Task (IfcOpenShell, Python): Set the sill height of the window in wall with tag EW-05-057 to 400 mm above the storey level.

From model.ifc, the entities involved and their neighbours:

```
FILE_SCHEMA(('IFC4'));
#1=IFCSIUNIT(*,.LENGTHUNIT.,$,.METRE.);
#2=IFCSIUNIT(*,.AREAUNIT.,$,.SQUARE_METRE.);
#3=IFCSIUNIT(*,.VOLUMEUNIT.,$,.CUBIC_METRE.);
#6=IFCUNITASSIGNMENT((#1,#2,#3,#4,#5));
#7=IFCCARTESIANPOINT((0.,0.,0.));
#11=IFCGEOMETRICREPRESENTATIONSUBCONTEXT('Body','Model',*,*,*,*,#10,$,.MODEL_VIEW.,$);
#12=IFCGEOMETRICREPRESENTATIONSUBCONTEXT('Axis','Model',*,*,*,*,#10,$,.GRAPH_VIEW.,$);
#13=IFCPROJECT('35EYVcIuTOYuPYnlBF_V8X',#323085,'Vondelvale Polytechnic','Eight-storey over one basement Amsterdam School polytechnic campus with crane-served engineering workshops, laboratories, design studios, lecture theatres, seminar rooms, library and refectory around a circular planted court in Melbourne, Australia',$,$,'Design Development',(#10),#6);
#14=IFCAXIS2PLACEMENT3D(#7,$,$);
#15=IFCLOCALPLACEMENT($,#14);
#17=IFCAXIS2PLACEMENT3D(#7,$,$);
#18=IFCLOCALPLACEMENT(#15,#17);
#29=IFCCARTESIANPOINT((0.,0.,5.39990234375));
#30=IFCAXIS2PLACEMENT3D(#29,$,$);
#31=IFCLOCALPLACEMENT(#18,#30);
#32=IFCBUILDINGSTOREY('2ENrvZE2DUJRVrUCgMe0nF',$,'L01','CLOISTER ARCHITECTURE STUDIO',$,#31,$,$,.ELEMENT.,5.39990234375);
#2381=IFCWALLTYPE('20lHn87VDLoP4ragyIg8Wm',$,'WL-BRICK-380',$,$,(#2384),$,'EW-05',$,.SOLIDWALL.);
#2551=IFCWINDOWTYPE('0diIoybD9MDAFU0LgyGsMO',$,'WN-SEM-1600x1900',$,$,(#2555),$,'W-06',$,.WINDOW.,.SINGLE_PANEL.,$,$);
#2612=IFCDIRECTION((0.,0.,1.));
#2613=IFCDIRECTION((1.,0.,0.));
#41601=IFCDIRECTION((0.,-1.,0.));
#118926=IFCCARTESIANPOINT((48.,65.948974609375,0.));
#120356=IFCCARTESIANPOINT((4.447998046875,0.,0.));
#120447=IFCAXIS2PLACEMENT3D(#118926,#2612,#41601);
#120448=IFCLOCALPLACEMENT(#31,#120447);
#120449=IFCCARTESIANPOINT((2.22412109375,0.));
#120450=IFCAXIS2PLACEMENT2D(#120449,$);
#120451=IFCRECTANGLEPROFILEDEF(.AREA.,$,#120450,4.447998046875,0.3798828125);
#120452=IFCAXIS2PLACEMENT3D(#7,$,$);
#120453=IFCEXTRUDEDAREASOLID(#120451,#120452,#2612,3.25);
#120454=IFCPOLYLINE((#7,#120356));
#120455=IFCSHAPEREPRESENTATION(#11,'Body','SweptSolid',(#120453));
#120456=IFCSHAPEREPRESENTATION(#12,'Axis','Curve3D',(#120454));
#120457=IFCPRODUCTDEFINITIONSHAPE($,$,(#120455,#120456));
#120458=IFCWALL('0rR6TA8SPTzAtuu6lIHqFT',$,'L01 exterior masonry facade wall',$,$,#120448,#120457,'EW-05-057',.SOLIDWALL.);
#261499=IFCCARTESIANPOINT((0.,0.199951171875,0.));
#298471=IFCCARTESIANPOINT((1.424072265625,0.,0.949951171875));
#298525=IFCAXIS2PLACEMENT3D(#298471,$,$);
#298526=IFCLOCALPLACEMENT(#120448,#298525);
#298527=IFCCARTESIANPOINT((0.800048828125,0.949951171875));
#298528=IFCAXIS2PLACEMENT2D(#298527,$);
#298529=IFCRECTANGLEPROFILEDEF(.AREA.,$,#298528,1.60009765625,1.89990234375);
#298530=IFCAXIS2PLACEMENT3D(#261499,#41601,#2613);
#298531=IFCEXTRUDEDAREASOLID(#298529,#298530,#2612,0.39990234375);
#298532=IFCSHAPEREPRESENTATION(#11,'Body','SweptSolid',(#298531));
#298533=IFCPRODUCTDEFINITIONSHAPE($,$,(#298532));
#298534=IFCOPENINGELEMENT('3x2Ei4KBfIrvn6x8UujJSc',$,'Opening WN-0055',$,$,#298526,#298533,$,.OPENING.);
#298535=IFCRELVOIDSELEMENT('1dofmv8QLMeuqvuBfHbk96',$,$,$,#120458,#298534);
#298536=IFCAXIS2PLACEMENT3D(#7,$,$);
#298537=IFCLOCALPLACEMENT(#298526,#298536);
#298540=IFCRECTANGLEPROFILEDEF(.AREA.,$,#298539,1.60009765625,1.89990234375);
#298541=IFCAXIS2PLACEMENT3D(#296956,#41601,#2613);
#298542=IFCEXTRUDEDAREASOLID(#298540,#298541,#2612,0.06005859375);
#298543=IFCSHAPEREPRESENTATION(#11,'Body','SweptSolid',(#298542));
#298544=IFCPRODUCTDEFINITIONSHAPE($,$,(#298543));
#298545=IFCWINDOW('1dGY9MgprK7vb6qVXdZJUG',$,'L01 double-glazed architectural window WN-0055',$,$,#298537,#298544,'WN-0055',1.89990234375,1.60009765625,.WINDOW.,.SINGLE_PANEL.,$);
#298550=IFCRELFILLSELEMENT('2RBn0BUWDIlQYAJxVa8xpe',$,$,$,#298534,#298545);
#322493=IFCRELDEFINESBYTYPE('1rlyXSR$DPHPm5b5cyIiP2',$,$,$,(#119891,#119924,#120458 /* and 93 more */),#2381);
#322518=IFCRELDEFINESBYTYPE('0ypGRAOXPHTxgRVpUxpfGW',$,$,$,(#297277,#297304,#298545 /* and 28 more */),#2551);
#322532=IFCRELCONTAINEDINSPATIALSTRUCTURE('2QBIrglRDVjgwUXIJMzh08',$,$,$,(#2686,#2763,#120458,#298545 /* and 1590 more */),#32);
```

```python
import numpy as np
import ifcopenshell
import ifcopenshell.api.geometry
import ifcopenshell.geom
import ifcopenshell.util.element
import ifcopenshell.util.placement
import ifcopenshell.util.shape
import ifcopenshell.util.unit

model = ifcopenshell.open("model.ifc")
unit_scale = ifcopenshell.util.unit.calculate_unit_scale(model)

window = model.by_guid("1dGY9MgprK7vb6qVXdZJUG")
opening = window.FillsVoids[0].RelatingOpeningElement
storey = ifcopenshell.util.element.get_container(window, ifc_class="IfcBuildingStorey")
level = ifcopenshell.util.placement.get_local_placement(storey.ObjectPlacement)[2, 3]

# The opening's origin need not be at the sill, so measure its lowest point.
shape = ifcopenshell.geom.create_shape(ifcopenshell.geom.settings(), opening)
bottom = ifcopenshell.util.shape.get_shape_bottom_elevation(shape, shape.geometry) / unit_scale
dz = level + 0.4 - bottom

shift = np.array([0.0, 0.0, dz])
# The window is placed relative to its opening, so it follows when the opening moves.
matrix = ifcopenshell.util.placement.get_local_placement(opening.ObjectPlacement)
matrix[:3, 3] += shift
ifcopenshell.api.geometry.edit_object_placement(
    model, product=opening, matrix=matrix, is_si=False, should_transform_children=True
)

print(f"moved by {dz * unit_scale:+.3f} m")

model.write("model_rev.ifc")
```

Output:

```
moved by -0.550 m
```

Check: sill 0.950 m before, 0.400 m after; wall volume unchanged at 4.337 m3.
